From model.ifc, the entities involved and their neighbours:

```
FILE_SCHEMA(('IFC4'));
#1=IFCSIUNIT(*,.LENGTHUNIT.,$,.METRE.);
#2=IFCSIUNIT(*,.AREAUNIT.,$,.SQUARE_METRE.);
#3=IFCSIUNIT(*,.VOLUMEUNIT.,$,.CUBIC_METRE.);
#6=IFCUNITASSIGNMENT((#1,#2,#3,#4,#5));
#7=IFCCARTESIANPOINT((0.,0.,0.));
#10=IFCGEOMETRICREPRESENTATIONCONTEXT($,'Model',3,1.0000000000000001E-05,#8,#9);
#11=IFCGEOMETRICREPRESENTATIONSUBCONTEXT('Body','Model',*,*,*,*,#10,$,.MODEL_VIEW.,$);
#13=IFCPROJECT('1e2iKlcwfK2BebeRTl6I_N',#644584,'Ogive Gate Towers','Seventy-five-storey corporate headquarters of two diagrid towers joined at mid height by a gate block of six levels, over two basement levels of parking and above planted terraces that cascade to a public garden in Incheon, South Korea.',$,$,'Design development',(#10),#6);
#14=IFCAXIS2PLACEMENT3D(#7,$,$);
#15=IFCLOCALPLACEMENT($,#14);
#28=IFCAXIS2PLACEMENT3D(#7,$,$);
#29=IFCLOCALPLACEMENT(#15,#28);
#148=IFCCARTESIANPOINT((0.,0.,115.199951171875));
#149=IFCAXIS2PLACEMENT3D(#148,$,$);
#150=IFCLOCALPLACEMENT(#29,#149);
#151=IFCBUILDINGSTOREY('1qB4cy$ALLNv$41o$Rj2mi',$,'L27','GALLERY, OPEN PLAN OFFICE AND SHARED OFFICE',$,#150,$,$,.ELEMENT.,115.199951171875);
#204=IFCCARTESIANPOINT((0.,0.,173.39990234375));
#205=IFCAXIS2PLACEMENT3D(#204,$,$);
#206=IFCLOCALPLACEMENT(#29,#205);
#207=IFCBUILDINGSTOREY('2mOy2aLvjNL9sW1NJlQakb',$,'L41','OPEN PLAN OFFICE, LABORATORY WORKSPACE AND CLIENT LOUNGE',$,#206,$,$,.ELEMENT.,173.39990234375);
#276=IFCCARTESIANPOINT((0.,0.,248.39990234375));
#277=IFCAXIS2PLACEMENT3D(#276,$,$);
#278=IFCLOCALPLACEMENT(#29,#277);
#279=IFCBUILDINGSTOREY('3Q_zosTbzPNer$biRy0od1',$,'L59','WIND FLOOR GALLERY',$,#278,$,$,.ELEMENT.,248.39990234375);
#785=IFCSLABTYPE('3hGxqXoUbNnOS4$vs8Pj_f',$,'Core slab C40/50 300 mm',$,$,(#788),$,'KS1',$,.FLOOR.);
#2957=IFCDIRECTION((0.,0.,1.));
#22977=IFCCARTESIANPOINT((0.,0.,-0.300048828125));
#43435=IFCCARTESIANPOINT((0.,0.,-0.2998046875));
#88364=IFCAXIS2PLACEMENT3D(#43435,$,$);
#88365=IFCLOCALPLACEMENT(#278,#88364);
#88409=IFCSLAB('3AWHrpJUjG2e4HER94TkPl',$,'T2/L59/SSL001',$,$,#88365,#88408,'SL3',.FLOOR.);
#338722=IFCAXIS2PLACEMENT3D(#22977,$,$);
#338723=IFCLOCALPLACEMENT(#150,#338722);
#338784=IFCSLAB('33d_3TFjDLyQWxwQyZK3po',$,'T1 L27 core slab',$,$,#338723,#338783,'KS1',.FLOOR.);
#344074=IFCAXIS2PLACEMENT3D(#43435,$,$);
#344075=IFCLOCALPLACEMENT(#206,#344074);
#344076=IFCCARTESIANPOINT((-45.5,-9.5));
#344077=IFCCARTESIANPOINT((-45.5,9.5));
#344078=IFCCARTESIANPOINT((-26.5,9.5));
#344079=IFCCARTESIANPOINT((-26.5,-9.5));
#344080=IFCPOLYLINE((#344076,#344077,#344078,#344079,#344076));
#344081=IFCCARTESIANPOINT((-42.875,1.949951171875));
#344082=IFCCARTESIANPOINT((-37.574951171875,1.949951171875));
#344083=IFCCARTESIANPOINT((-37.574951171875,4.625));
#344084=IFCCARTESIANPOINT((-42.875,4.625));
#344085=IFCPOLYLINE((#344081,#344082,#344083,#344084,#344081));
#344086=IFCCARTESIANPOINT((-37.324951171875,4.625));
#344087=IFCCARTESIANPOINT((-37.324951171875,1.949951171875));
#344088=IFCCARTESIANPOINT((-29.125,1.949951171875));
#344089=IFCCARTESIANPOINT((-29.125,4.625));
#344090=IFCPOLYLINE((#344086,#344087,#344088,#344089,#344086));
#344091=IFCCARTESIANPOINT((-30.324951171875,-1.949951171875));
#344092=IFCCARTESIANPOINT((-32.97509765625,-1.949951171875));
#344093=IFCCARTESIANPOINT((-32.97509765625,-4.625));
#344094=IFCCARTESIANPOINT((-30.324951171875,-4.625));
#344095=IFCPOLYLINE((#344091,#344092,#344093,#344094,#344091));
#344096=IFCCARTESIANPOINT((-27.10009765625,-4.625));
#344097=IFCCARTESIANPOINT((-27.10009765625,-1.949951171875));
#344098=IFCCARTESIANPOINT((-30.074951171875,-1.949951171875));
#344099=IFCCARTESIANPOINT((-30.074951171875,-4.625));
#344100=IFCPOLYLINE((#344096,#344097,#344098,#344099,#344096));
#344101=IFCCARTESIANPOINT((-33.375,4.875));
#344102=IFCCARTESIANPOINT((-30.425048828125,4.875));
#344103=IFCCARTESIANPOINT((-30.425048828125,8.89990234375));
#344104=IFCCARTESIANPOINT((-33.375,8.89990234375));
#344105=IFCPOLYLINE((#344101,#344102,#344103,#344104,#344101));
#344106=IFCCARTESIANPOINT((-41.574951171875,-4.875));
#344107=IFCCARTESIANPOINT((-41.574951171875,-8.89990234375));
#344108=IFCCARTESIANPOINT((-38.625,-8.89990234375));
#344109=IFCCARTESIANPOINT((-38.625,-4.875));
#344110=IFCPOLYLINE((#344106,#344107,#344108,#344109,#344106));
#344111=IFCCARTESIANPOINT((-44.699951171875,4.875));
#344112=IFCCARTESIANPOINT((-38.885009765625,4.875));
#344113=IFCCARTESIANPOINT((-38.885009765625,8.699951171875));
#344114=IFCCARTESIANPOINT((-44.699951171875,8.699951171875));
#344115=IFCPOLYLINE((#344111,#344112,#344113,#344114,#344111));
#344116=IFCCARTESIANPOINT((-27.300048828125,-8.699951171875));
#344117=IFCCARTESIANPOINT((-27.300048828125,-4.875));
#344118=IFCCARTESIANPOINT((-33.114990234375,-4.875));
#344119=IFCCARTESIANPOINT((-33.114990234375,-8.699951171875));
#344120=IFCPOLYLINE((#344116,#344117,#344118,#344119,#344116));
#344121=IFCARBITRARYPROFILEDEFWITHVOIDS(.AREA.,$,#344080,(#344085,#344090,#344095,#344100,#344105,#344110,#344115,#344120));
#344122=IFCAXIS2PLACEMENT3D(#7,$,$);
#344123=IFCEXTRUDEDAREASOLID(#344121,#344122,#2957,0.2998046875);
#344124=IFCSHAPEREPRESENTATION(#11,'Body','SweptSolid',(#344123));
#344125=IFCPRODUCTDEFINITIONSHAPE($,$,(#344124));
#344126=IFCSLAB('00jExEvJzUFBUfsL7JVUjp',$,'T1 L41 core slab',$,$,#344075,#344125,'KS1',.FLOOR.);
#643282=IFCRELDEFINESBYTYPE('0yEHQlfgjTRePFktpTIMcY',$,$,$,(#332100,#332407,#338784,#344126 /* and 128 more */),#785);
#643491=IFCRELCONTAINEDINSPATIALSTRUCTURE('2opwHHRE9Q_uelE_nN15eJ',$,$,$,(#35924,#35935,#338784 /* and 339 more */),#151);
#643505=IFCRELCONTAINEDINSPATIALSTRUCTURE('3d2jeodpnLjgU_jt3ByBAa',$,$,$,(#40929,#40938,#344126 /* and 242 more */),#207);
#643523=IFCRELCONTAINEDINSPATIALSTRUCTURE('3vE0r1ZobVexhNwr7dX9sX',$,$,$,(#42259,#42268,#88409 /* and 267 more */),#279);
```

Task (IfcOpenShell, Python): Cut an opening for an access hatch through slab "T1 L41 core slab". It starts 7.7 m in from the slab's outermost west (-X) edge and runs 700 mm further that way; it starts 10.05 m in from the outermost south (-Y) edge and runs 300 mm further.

```python
import numpy as np
import ifcopenshell
import ifcopenshell.api.feature
import ifcopenshell.api.geometry
import ifcopenshell.api.root
import ifcopenshell.geom
import ifcopenshell.util.placement
import ifcopenshell.util.representation
import ifcopenshell.util.shape
import ifcopenshell.util.unit

model = ifcopenshell.open("model.ifc")
unit_scale = ifcopenshell.util.unit.calculate_unit_scale(model)
settings = ifcopenshell.geom.settings()


def volume(element):
    """Net volume in cubic metres, openings subtracted."""
    shape = ifcopenshell.geom.create_shape(settings, element)
    return ifcopenshell.util.shape.get_volume(shape.geometry)


slab = model.by_guid("00jExEvJzUFBUfsL7JVUjp")
before = volume(slab)

# Extent in the slab's own axes, in metres. The edges named are its -X and -Y sides.
slab_shape = ifcopenshell.geom.create_shape(settings, slab)
vertices = ifcopenshell.util.shape.get_vertices(slab_shape.geometry)
x_min, y_min, bottom = vertices.min(axis=0)
top = vertices[:, 2].max()

opening = ifcopenshell.api.root.create_entity(model, ifc_class="IfcOpeningElement", name="Access hatch opening", predefined_type="OPENING")
context = ifcopenshell.util.representation.get_context(model, "Model", "Body", "MODEL_VIEW")
width, depth = 0.7, 0.3
outline = [(0.0, 0.0), (width, 0.0), (width, depth), (0.0, depth), (0.0, 0.0)]
# Overshoot both faces by 50 mm so the cut is clean.
shape = ifcopenshell.api.geometry.add_slab_representation(
    model, context=context, depth=top - bottom + 0.1, polyline=outline
)
ifcopenshell.api.geometry.assign_representation(model, product=opening, representation=shape)

matrix = ifcopenshell.util.placement.get_local_placement(slab.ObjectPlacement)
matrix[:, 3] = matrix @ np.append(np.array([x_min + 7.7, y_min + 10.05, bottom - 0.05]) / unit_scale, 1.0)
ifcopenshell.api.geometry.edit_object_placement(model, product=opening, matrix=matrix, is_si=False)
ifcopenshell.api.feature.add_feature(model, feature=opening, element=slab)

after = volume(slab)

print(f"slab volume {before:.3f} -> {after:.3f} m3")

model.write("model_rev.ifc")
```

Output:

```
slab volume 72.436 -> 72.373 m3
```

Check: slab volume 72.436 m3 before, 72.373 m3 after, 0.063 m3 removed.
